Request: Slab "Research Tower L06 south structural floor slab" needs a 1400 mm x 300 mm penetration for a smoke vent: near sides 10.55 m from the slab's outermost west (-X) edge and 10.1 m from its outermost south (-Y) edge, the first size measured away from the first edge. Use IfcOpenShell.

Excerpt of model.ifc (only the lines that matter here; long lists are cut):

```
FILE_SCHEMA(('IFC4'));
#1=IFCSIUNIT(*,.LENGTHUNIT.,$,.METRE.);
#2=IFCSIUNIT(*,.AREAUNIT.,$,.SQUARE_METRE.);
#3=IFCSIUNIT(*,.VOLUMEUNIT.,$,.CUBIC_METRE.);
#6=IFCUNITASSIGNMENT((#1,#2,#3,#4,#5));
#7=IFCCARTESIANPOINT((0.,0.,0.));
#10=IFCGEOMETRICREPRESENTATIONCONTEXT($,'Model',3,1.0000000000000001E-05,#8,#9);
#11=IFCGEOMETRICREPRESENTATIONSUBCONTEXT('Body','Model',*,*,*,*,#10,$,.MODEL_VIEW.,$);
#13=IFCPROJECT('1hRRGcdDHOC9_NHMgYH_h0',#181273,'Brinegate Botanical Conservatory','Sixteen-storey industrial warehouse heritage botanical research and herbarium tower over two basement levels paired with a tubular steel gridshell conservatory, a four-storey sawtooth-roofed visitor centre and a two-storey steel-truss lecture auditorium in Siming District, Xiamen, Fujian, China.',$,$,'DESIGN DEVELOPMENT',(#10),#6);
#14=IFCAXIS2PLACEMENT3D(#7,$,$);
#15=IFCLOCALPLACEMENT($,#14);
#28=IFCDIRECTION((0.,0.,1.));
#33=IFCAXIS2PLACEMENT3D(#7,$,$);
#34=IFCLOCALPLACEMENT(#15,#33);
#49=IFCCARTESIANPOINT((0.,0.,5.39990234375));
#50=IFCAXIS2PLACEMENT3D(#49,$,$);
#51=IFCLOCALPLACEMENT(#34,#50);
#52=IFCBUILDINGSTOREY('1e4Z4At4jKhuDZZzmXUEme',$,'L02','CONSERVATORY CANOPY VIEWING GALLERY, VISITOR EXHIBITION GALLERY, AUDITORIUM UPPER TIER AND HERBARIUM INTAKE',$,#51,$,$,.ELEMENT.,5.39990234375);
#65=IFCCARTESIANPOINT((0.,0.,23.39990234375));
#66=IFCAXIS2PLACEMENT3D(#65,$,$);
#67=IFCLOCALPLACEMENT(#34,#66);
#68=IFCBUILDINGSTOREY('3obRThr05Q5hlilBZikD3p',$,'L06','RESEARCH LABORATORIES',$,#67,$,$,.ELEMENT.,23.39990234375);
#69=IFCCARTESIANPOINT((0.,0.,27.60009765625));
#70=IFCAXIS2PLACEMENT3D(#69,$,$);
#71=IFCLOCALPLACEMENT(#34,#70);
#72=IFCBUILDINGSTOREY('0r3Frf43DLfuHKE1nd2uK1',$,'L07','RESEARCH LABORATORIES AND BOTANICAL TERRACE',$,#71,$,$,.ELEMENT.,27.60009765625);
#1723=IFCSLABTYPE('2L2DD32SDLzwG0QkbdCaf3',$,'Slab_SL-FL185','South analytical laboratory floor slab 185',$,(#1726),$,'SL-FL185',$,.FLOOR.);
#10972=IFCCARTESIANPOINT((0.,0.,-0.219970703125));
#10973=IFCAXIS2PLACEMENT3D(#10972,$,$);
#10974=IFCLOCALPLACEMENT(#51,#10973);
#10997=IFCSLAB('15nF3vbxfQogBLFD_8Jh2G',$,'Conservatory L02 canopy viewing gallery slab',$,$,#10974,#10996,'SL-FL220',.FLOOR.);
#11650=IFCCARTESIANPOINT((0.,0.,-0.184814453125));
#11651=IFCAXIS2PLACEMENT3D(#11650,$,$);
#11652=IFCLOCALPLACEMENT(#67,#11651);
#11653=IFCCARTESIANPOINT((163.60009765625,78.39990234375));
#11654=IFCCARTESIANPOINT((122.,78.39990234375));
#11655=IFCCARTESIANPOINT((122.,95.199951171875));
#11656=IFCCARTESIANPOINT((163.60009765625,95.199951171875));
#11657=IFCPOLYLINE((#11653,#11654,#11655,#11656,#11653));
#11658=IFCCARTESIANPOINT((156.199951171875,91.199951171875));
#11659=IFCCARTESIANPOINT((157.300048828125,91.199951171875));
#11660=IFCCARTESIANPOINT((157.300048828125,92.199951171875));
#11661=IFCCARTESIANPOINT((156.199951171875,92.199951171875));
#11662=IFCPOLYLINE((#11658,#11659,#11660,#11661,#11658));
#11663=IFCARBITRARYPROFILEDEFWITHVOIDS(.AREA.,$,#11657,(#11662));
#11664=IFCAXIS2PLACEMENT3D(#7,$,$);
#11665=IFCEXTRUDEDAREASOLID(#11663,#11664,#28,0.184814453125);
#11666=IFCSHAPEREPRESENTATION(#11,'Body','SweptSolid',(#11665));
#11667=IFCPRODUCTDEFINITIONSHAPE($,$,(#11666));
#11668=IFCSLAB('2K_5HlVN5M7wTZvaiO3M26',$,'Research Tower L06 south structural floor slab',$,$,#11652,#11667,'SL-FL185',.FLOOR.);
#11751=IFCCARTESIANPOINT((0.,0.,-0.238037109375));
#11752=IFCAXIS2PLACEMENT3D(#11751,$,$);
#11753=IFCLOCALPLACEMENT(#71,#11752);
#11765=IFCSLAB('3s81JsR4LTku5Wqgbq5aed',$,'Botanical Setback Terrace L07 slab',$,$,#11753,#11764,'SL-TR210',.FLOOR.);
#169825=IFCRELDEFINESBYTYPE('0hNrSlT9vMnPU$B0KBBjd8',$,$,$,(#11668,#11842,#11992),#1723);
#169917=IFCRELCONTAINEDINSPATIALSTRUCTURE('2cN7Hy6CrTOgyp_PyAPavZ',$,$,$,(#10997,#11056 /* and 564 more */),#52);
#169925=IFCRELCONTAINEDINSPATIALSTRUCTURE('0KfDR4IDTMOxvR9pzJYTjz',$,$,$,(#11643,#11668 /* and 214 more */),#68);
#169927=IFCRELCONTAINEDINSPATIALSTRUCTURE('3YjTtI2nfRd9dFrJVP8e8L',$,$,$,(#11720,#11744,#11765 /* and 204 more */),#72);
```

```python
import numpy as np
import ifcopenshell
import ifcopenshell.api.feature
import ifcopenshell.api.geometry
import ifcopenshell.api.root
import ifcopenshell.geom
import ifcopenshell.util.placement
import ifcopenshell.util.representation
import ifcopenshell.util.shape
import ifcopenshell.util.unit

model = ifcopenshell.open("model.ifc")
unit_scale = ifcopenshell.util.unit.calculate_unit_scale(model)
settings = ifcopenshell.geom.settings()


def volume(element):
    """Net volume in cubic metres, openings subtracted."""
    shape = ifcopenshell.geom.create_shape(settings, element)
    return ifcopenshell.util.shape.get_volume(shape.geometry)


slab = model.by_guid("2K_5HlVN5M7wTZvaiO3M26")
before = volume(slab)

# Extent in the slab's own axes, in metres. The edges named are its -X and -Y sides.
slab_shape = ifcopenshell.geom.create_shape(settings, slab)
vertices = ifcopenshell.util.shape.get_vertices(slab_shape.geometry)
x_min, y_min, bottom = vertices.min(axis=0)
top = vertices[:, 2].max()

opening = ifcopenshell.api.root.create_entity(model, ifc_class="IfcOpeningElement", name="Smoke vent opening", predefined_type="OPENING")
context = ifcopenshell.util.representation.get_context(model, "Model", "Body", "MODEL_VIEW")
width, depth = 1.4, 0.3
outline = [(0.0, 0.0), (width, 0.0), (width, depth), (0.0, depth), (0.0, 0.0)]
# Overshoot both faces by 50 mm so the cut is clean.
shape = ifcopenshell.api.geometry.add_slab_representation(
    model, context=context, depth=top - bottom + 0.1, polyline=outline
)
ifcopenshell.api.geometry.assign_representation(model, product=opening, representation=shape)

matrix = ifcopenshell.util.placement.get_local_placement(slab.ObjectPlacement)
matrix[:, 3] = matrix @ np.append(np.array([x_min + 10.55, y_min + 10.1, bottom - 0.05]) / unit_scale, 1.0)
ifcopenshell.api.geometry.edit_object_placement(model, product=opening, matrix=matrix, is_si=False)
ifcopenshell.api.feature.add_feature(model, feature=opening, element=slab)

after = volume(slab)

print(f"slab volume {before:.3f} -> {after:.3f} m3")

model.write("model-out.ifc")
```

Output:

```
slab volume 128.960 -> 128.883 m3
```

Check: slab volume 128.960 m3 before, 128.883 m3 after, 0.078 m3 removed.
